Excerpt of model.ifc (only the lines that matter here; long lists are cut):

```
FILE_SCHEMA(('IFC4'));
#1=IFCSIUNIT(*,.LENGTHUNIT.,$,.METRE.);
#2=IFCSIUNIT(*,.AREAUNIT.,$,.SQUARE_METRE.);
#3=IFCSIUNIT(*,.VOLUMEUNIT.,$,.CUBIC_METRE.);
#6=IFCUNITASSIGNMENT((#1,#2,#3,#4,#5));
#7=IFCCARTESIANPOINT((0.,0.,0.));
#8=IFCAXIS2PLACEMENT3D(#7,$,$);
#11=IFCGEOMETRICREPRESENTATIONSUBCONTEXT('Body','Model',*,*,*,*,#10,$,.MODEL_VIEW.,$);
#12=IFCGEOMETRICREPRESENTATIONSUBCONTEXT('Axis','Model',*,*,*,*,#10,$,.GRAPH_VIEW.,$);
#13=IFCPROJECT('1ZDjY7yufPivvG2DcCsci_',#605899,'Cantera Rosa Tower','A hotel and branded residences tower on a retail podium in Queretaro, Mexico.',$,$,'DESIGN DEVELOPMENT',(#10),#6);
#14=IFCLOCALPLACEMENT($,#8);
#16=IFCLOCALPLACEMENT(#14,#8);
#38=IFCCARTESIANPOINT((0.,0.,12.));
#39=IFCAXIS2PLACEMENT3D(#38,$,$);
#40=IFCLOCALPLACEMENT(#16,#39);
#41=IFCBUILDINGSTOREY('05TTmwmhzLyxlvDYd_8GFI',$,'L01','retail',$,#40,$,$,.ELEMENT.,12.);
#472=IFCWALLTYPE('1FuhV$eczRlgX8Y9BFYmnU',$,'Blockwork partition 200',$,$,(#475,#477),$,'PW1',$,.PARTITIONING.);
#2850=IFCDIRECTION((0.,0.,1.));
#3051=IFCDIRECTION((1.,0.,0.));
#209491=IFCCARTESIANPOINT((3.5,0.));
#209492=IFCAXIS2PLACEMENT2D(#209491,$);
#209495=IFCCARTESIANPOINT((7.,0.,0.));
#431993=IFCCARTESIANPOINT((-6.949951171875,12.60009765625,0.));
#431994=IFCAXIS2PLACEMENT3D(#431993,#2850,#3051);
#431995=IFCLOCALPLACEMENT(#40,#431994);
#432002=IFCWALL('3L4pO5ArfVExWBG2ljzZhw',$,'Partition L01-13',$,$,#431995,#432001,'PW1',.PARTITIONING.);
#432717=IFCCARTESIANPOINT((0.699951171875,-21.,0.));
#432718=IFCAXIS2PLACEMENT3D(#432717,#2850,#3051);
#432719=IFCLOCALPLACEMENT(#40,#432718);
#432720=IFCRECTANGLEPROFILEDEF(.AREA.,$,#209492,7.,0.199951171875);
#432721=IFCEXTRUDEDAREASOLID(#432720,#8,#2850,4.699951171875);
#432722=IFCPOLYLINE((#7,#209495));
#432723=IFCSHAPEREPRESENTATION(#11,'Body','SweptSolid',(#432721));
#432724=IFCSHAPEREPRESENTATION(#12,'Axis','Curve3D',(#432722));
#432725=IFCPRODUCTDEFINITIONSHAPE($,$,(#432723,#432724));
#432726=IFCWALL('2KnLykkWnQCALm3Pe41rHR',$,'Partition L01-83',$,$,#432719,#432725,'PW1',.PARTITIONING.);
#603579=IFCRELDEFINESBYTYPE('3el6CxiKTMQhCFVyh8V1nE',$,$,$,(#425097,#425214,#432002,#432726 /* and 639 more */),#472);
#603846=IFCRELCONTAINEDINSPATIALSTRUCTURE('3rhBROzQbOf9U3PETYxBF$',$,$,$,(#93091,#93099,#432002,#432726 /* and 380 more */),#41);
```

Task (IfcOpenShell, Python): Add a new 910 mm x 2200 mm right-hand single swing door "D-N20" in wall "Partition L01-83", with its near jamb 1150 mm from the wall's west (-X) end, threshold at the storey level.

```python
import numpy as np
import ifcopenshell
import ifcopenshell.api.feature
import ifcopenshell.api.geometry
import ifcopenshell.api.root
import ifcopenshell.api.spatial
import ifcopenshell.geom
import ifcopenshell.util.element
import ifcopenshell.util.placement
import ifcopenshell.util.representation
import ifcopenshell.util.shape
import ifcopenshell.util.unit

model = ifcopenshell.open("model.ifc")
unit_scale = ifcopenshell.util.unit.calculate_unit_scale(model)
settings = ifcopenshell.geom.settings()


def volume(element):
    """Net volume in cubic metres, openings subtracted."""
    shape = ifcopenshell.geom.create_shape(settings, element)
    return ifcopenshell.util.shape.get_volume(shape.geometry)


wall = model.by_guid("2KnLykkWnQCALm3Pe41rHR")
storey = ifcopenshell.util.element.get_container(wall, ifc_class="IfcBuildingStorey")
context = ifcopenshell.util.representation.get_context(model, "Model", "Body", "MODEL_VIEW")
before = volume(wall)

width, height, from_end, sill = 0.91, 2.2, 1.15, 0.0  # metres

# The wall runs along its own X axis, and the end named is its -X end.
wall_shape = ifcopenshell.geom.create_shape(settings, wall)
x, y, z = ifcopenshell.util.shape.get_vertices(wall_shape.geometry).T
start = x.min() + from_end
face, thickness = float(y.min()), float(y.max() - y.min())
wall_matrix = ifcopenshell.util.placement.get_local_placement(wall.ObjectPlacement)
level = ifcopenshell.util.placement.get_local_placement(storey.ObjectPlacement)[2, 3]


def in_wall(x, y):
    """Placement at x, y metres in the wall's axes, at sill height."""
    matrix = wall_matrix.copy()
    matrix[:, 3] = wall_matrix @ np.array([x / unit_scale, y / unit_scale, 0.0, 1.0])
    matrix[2, 3] = level + sill / unit_scale
    return matrix


# Opening: a box that overshoots both wall faces by 50 mm.
opening = ifcopenshell.api.root.create_entity(model, ifc_class="IfcOpeningElement", predefined_type="OPENING")
box = ifcopenshell.api.geometry.add_wall_representation(
    model, context=context, length=width, height=height, thickness=thickness + 0.1
)
ifcopenshell.api.geometry.assign_representation(model, product=opening, representation=box)
ifcopenshell.api.geometry.edit_object_placement(model, product=opening, matrix=in_wall(start, face - 0.05), is_si=False)
ifcopenshell.api.feature.add_feature(model, feature=opening, element=wall)

door = ifcopenshell.api.root.create_entity(model, ifc_class="IfcDoor", name="D-N20", predefined_type="DOOR")
door.OverallWidth, door.OverallHeight = width / unit_scale, height / unit_scale
door.OperationType = "SINGLE_SWING_RIGHT"
body = ifcopenshell.api.geometry.add_door_representation(
    model,
    context=context,
    overall_width=door.OverallWidth,
    overall_height=door.OverallHeight,
    operation_type="SINGLE_SWING_RIGHT",
    lining_properties={"LiningDepth": thickness / unit_scale, "ThresholdDepth": thickness / unit_scale},
)
ifcopenshell.api.geometry.assign_representation(model, product=door, representation=body)
ifcopenshell.api.spatial.assign_container(model, products=[door], relating_structure=storey)
ifcopenshell.api.feature.add_filling(model, opening=opening, element=door)

# The lining spans the wall, so the door starts at the wall face.
ifcopenshell.api.geometry.edit_object_placement(model, product=door, matrix=in_wall(start, face), is_si=False)

after = volume(wall)

print(f"wall volume {before:.3f} -> {after:.3f} m3")

model.write("model_edited.ifc")
```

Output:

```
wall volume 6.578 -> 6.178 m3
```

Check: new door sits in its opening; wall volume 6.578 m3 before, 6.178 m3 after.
